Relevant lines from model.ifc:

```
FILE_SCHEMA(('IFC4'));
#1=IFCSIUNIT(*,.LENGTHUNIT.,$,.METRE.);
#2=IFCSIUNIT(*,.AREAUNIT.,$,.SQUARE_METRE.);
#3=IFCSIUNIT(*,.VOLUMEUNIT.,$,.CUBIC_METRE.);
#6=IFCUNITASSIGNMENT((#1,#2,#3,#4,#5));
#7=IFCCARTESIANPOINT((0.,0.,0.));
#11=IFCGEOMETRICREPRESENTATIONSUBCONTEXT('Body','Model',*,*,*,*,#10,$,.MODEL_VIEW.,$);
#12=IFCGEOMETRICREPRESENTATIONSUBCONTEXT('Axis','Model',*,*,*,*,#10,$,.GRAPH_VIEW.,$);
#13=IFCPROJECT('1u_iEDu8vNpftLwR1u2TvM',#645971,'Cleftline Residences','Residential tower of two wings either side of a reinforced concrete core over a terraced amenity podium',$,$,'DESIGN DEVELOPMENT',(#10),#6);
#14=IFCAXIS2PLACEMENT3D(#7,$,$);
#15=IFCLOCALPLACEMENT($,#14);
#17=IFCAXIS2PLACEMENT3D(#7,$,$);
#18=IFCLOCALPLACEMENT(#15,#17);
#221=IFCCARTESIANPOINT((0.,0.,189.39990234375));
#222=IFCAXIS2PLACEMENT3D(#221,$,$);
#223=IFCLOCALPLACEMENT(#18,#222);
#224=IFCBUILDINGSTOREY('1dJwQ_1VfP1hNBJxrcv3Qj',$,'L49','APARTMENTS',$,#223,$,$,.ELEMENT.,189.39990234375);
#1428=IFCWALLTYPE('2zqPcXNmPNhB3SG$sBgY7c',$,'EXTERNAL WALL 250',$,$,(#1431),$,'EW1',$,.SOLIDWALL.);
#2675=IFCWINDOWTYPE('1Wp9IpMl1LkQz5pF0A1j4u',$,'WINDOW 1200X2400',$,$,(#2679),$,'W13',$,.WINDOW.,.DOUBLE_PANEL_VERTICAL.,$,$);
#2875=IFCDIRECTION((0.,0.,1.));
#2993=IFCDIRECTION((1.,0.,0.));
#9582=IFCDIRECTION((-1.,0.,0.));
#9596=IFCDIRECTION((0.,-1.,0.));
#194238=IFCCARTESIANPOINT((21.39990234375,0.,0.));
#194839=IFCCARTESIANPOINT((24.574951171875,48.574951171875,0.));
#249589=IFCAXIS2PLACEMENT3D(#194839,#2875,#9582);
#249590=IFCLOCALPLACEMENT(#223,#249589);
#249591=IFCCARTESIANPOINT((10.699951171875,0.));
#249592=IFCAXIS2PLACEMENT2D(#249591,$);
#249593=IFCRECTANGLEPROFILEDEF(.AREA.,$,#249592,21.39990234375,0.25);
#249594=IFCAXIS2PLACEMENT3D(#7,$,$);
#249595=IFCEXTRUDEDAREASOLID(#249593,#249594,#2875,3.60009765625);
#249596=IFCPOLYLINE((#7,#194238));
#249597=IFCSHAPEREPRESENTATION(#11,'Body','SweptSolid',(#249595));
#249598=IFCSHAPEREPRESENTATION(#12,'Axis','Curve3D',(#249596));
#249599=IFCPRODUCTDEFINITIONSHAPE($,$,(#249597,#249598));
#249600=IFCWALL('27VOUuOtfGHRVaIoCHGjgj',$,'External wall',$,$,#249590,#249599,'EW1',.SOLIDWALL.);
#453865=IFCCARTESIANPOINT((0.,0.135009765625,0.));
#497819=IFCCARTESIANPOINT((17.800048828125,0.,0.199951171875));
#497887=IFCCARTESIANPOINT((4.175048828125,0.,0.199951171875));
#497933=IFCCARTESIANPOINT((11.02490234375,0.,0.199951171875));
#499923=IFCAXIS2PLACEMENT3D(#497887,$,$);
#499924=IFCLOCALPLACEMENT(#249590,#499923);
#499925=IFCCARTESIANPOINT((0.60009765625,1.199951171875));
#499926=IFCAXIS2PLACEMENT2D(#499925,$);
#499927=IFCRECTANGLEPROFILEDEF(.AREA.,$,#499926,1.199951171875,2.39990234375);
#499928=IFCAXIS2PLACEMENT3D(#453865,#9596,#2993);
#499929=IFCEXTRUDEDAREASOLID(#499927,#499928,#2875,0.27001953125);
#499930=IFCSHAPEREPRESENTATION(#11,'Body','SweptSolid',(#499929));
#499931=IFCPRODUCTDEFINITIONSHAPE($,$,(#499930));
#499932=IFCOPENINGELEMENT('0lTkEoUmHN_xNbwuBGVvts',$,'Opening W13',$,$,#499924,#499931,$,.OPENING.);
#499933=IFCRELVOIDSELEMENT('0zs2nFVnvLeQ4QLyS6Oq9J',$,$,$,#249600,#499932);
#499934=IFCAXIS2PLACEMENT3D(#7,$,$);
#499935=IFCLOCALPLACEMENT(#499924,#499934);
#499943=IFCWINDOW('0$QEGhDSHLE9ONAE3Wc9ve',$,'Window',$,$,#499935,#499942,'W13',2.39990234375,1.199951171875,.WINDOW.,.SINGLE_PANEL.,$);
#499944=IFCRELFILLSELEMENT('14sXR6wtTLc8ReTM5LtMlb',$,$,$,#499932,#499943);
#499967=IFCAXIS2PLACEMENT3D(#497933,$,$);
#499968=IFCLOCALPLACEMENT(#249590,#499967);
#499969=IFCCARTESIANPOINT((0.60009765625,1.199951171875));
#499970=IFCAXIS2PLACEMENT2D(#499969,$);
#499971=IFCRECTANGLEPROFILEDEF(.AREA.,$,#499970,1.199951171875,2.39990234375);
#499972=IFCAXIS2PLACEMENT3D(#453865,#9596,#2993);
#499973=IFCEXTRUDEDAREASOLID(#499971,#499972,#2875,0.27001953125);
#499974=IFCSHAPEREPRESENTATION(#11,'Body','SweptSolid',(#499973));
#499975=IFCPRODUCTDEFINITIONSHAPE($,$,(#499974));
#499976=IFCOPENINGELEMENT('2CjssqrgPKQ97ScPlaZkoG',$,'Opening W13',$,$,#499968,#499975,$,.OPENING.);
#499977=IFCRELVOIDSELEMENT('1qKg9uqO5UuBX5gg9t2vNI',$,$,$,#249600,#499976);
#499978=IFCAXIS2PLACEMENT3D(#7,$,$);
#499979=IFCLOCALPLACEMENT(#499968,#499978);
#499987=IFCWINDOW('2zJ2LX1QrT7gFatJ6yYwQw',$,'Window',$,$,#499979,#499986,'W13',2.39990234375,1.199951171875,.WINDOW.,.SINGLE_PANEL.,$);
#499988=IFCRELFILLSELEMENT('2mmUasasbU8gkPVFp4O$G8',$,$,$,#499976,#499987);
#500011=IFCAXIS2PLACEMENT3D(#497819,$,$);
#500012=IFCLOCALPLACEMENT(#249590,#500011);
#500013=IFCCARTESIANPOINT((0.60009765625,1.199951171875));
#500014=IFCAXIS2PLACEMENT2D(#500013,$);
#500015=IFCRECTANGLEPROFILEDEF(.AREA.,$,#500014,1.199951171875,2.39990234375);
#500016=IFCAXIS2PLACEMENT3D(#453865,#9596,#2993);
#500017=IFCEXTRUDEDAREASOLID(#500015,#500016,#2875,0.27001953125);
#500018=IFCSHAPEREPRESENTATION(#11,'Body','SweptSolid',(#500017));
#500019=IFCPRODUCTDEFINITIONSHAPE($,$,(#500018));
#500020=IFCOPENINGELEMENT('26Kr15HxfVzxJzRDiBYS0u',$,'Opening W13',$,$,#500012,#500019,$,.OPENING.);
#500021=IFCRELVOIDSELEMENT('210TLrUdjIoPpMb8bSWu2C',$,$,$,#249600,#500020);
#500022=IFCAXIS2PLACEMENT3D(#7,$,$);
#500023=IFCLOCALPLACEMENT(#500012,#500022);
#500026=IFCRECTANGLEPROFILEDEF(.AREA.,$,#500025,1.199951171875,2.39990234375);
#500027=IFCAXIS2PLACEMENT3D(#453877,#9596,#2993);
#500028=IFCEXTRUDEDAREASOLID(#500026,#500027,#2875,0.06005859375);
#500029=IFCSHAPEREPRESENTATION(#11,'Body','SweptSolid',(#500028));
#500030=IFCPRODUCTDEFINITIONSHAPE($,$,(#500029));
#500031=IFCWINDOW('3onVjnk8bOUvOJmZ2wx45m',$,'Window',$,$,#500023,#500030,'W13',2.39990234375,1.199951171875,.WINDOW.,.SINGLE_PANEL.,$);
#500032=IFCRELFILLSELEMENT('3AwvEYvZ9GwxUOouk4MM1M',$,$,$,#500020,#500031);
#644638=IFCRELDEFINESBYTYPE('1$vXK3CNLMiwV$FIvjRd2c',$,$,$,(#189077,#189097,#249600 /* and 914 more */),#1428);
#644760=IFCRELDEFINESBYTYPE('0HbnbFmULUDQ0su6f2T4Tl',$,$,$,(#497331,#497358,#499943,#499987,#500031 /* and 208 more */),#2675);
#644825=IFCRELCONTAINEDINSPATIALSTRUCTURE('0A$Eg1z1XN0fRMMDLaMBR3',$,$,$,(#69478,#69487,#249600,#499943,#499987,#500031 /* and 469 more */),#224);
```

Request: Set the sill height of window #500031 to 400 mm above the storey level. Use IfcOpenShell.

```python
import numpy as np
import ifcopenshell
import ifcopenshell.api.geometry
import ifcopenshell.geom
import ifcopenshell.util.element
import ifcopenshell.util.placement
import ifcopenshell.util.shape
import ifcopenshell.util.unit

model = ifcopenshell.open("model.ifc")
unit_scale = ifcopenshell.util.unit.calculate_unit_scale(model)

window = model.by_guid("3onVjnk8bOUvOJmZ2wx45m")
opening = window.FillsVoids[0].RelatingOpeningElement
storey = ifcopenshell.util.element.get_container(window, ifc_class="IfcBuildingStorey")
level = ifcopenshell.util.placement.get_local_placement(storey.ObjectPlacement)[2, 3]

# The opening's origin need not be at the sill, so measure its lowest point.
shape = ifcopenshell.geom.create_shape(ifcopenshell.geom.settings(), opening)
bottom = ifcopenshell.util.shape.get_shape_bottom_elevation(shape, shape.geometry) / unit_scale
dz = level + 0.4 / unit_scale - bottom

shift = np.array([0.0, 0.0, dz])
# The window is placed relative to its opening, so it follows when the opening moves.
matrix = ifcopenshell.util.placement.get_local_placement(opening.ObjectPlacement)
matrix[:3, 3] += shift
ifcopenshell.api.geometry.edit_object_placement(
    model, product=opening, matrix=matrix, is_si=False, should_transform_children=True
)

print(f"moved by {dz * unit_scale:+.3f} m")

model.write("model_v2.ifc")
```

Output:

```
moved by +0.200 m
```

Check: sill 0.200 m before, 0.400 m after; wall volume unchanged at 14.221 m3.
